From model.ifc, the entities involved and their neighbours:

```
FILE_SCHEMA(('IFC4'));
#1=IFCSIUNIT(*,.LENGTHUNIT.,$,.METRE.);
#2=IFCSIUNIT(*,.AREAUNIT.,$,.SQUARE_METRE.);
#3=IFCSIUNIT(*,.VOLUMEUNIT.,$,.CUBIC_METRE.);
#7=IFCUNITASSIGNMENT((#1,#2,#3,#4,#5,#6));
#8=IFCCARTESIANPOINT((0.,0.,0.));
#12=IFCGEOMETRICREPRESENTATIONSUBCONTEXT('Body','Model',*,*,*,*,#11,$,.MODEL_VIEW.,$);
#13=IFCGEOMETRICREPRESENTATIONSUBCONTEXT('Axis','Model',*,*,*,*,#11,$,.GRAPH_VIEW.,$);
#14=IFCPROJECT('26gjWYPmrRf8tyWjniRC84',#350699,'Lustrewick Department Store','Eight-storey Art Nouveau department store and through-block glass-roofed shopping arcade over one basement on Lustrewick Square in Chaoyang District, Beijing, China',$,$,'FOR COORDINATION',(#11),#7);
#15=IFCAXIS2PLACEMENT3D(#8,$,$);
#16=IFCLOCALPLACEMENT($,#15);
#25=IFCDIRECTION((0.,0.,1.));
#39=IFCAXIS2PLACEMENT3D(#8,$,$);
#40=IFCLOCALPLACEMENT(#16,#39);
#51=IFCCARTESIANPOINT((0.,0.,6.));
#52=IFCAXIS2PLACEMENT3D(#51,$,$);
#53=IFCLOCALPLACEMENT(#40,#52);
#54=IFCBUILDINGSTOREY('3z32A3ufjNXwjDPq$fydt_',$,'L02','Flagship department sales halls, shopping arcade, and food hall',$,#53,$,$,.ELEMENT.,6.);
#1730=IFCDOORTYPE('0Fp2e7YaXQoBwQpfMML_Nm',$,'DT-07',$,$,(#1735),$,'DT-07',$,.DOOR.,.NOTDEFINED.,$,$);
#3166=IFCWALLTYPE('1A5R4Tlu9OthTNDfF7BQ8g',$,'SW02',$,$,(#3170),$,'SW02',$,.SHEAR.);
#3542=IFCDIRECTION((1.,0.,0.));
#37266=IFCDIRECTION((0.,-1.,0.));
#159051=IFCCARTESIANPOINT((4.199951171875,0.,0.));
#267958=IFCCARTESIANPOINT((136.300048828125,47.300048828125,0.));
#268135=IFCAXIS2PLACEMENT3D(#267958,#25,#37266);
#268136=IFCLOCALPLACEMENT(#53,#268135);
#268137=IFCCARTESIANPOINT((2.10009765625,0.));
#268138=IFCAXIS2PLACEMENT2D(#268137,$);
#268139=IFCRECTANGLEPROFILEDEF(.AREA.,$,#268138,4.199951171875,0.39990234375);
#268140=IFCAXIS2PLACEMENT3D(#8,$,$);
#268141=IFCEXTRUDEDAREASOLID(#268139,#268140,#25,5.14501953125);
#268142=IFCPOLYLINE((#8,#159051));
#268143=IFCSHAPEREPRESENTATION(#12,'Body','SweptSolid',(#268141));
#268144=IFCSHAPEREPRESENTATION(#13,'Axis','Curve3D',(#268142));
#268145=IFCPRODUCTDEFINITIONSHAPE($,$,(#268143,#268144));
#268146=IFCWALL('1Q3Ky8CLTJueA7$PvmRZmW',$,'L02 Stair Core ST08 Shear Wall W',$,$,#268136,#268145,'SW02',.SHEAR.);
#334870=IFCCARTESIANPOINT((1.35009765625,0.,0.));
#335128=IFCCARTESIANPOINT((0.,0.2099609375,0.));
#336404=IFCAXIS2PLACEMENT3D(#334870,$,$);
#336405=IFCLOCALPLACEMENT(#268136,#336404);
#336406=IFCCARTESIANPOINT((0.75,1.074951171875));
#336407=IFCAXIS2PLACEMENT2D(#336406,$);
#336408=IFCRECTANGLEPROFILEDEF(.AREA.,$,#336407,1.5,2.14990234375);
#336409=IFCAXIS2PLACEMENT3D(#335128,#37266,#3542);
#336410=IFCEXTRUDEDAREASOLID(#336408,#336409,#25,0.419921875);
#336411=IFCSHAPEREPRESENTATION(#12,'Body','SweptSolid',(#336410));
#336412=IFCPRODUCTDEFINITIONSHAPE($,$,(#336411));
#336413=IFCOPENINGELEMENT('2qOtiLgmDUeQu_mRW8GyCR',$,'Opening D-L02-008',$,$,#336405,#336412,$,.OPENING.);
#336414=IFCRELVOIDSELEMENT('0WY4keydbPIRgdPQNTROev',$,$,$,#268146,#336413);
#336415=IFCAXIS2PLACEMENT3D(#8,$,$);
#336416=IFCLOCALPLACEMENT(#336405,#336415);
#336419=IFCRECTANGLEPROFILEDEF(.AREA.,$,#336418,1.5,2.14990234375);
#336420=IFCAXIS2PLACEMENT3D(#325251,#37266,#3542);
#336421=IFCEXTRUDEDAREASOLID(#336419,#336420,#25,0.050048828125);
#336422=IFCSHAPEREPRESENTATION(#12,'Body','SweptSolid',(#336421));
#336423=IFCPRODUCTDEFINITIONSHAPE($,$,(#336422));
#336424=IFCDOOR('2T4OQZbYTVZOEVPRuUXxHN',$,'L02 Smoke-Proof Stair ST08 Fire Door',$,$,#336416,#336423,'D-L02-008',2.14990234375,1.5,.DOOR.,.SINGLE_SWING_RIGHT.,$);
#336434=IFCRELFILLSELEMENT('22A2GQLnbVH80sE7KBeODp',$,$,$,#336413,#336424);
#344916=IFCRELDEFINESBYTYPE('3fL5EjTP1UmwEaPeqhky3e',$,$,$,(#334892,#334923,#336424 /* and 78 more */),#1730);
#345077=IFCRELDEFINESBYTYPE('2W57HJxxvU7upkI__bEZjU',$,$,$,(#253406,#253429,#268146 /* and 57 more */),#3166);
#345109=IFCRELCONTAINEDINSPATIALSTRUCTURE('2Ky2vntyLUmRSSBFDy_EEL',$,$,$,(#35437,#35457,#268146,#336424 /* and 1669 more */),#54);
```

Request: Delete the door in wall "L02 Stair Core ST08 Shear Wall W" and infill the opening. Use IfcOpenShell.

```python
import ifcopenshell
import ifcopenshell.api.feature
import ifcopenshell.api.root
import ifcopenshell.geom
import ifcopenshell.util.shape

model = ifcopenshell.open("model.ifc")
settings = ifcopenshell.geom.settings()


def volume(element):
    """Net volume in cubic metres, openings subtracted."""
    shape = ifcopenshell.geom.create_shape(settings, element)
    return ifcopenshell.util.shape.get_volume(shape.geometry)


door = model.by_guid("2T4OQZbYTVZOEVPRuUXxHN")
opening = door.FillsVoids[0].RelatingOpeningElement
wall = opening.VoidsElements[0].RelatingBuildingElement
before = volume(wall)

ifcopenshell.api.root.remove_product(model, product=door)
ifcopenshell.api.feature.remove_feature(model, feature=opening)

after = volume(wall)

print(f"wall volume {before:.3f} -> {after:.3f} m3")

model.write("model_rev.ifc")
```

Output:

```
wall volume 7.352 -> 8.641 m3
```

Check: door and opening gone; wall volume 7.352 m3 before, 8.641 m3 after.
